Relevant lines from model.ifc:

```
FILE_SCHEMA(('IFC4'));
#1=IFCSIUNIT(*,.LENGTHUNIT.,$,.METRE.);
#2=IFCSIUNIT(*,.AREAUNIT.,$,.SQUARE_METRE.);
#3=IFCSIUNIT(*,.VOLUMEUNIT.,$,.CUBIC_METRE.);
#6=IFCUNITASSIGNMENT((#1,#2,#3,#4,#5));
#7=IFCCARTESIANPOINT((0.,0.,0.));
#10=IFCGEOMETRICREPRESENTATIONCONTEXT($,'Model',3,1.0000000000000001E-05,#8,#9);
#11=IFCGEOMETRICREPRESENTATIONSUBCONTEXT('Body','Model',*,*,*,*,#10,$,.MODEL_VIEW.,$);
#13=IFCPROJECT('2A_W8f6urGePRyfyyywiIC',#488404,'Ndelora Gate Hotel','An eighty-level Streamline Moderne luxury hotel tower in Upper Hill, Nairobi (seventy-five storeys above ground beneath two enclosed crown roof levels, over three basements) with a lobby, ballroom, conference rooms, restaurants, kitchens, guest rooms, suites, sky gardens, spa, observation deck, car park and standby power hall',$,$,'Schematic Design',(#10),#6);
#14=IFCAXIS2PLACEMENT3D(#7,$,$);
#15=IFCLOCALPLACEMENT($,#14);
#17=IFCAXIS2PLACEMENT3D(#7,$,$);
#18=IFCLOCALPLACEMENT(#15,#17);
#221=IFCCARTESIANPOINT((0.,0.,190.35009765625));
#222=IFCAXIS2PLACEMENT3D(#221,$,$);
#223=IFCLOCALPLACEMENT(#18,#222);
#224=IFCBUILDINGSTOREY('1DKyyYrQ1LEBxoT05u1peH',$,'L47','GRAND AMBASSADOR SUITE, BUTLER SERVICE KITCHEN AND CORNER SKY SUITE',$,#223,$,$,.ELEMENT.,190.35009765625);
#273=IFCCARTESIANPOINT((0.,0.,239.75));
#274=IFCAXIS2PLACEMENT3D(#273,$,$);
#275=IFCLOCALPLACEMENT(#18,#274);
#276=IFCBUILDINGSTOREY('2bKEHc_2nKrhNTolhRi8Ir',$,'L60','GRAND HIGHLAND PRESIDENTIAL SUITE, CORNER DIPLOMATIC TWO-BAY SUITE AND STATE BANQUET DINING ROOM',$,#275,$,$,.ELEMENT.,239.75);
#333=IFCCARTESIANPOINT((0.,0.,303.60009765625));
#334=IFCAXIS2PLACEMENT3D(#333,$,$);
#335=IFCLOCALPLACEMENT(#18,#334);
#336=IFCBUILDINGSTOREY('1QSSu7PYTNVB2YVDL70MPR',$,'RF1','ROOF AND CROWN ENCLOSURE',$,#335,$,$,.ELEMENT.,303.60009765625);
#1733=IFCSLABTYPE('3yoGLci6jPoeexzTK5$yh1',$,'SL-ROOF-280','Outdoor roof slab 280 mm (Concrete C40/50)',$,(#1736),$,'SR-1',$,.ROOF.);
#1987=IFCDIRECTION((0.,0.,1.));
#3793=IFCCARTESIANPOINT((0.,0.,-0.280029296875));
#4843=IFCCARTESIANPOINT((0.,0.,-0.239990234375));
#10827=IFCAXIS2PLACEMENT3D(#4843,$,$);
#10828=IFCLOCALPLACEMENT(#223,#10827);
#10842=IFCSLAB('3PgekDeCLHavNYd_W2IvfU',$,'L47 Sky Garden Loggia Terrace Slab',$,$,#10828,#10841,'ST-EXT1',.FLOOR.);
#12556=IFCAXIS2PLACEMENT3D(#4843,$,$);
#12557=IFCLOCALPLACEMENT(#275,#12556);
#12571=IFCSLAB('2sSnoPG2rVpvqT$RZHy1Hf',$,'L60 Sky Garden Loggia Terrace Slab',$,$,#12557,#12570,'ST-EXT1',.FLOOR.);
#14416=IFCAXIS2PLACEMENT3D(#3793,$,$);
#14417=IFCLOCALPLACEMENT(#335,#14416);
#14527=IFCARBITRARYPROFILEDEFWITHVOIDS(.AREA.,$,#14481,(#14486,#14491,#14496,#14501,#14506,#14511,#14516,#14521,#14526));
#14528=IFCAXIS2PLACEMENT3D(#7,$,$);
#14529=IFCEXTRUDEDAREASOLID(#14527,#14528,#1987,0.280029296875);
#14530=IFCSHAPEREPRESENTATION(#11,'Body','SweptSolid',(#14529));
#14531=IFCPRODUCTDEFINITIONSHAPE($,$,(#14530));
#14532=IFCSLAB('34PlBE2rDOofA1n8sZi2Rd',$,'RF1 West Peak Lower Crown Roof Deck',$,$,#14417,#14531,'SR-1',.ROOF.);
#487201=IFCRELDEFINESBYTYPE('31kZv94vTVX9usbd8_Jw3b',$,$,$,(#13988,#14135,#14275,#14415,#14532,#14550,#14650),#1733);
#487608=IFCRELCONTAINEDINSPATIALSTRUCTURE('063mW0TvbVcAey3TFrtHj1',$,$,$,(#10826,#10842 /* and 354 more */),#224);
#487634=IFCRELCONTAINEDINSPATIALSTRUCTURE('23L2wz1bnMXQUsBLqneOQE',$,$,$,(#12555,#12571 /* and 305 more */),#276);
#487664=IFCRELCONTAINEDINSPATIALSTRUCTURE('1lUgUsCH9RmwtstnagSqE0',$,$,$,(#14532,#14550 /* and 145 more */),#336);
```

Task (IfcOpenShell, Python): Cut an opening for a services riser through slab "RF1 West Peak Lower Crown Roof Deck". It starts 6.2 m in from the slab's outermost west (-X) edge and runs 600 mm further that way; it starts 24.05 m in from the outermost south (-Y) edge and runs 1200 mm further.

```python
import numpy as np
import ifcopenshell
import ifcopenshell.api.feature
import ifcopenshell.api.geometry
import ifcopenshell.api.root
import ifcopenshell.geom
import ifcopenshell.util.placement
import ifcopenshell.util.representation
import ifcopenshell.util.shape
import ifcopenshell.util.unit

model = ifcopenshell.open("model.ifc")
unit_scale = ifcopenshell.util.unit.calculate_unit_scale(model)
settings = ifcopenshell.geom.settings()


def volume(element):
    """Net volume in cubic metres, openings subtracted."""
    shape = ifcopenshell.geom.create_shape(settings, element)
    return ifcopenshell.util.shape.get_volume(shape.geometry)


slab = model.by_guid("34PlBE2rDOofA1n8sZi2Rd")
before = volume(slab)

# Extent in the slab's own axes, in metres. The edges named are its -X and -Y sides.
slab_shape = ifcopenshell.geom.create_shape(settings, slab)
vertices = ifcopenshell.util.shape.get_vertices(slab_shape.geometry)
x_min, y_min, bottom = vertices.min(axis=0)
top = vertices[:, 2].max()

opening = ifcopenshell.api.root.create_entity(model, ifc_class="IfcOpeningElement", name="Services riser opening", predefined_type="OPENING")
context = ifcopenshell.util.representation.get_context(model, "Model", "Body", "MODEL_VIEW")
width, depth = 0.6, 1.2
outline = [(0.0, 0.0), (width, 0.0), (width, depth), (0.0, depth), (0.0, 0.0)]
# Overshoot both faces by 50 mm so the cut is clean.
shape = ifcopenshell.api.geometry.add_slab_representation(
    model, context=context, depth=top - bottom + 0.1, polyline=outline
)
ifcopenshell.api.geometry.assign_representation(model, product=opening, representation=shape)

matrix = ifcopenshell.util.placement.get_local_placement(slab.ObjectPlacement)
matrix[:, 3] = matrix @ np.append(np.array([x_min + 6.2, y_min + 24.05, bottom - 0.05]) / unit_scale, 1.0)
ifcopenshell.api.geometry.edit_object_placement(model, product=opening, matrix=matrix, is_si=False)
ifcopenshell.api.feature.add_feature(model, feature=opening, element=slab)

after = volume(slab)

print(f"slab volume {before:.3f} -> {after:.3f} m3")

model.write("model-out.ifc")
```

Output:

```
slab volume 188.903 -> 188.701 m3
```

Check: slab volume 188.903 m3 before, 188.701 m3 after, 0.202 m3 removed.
